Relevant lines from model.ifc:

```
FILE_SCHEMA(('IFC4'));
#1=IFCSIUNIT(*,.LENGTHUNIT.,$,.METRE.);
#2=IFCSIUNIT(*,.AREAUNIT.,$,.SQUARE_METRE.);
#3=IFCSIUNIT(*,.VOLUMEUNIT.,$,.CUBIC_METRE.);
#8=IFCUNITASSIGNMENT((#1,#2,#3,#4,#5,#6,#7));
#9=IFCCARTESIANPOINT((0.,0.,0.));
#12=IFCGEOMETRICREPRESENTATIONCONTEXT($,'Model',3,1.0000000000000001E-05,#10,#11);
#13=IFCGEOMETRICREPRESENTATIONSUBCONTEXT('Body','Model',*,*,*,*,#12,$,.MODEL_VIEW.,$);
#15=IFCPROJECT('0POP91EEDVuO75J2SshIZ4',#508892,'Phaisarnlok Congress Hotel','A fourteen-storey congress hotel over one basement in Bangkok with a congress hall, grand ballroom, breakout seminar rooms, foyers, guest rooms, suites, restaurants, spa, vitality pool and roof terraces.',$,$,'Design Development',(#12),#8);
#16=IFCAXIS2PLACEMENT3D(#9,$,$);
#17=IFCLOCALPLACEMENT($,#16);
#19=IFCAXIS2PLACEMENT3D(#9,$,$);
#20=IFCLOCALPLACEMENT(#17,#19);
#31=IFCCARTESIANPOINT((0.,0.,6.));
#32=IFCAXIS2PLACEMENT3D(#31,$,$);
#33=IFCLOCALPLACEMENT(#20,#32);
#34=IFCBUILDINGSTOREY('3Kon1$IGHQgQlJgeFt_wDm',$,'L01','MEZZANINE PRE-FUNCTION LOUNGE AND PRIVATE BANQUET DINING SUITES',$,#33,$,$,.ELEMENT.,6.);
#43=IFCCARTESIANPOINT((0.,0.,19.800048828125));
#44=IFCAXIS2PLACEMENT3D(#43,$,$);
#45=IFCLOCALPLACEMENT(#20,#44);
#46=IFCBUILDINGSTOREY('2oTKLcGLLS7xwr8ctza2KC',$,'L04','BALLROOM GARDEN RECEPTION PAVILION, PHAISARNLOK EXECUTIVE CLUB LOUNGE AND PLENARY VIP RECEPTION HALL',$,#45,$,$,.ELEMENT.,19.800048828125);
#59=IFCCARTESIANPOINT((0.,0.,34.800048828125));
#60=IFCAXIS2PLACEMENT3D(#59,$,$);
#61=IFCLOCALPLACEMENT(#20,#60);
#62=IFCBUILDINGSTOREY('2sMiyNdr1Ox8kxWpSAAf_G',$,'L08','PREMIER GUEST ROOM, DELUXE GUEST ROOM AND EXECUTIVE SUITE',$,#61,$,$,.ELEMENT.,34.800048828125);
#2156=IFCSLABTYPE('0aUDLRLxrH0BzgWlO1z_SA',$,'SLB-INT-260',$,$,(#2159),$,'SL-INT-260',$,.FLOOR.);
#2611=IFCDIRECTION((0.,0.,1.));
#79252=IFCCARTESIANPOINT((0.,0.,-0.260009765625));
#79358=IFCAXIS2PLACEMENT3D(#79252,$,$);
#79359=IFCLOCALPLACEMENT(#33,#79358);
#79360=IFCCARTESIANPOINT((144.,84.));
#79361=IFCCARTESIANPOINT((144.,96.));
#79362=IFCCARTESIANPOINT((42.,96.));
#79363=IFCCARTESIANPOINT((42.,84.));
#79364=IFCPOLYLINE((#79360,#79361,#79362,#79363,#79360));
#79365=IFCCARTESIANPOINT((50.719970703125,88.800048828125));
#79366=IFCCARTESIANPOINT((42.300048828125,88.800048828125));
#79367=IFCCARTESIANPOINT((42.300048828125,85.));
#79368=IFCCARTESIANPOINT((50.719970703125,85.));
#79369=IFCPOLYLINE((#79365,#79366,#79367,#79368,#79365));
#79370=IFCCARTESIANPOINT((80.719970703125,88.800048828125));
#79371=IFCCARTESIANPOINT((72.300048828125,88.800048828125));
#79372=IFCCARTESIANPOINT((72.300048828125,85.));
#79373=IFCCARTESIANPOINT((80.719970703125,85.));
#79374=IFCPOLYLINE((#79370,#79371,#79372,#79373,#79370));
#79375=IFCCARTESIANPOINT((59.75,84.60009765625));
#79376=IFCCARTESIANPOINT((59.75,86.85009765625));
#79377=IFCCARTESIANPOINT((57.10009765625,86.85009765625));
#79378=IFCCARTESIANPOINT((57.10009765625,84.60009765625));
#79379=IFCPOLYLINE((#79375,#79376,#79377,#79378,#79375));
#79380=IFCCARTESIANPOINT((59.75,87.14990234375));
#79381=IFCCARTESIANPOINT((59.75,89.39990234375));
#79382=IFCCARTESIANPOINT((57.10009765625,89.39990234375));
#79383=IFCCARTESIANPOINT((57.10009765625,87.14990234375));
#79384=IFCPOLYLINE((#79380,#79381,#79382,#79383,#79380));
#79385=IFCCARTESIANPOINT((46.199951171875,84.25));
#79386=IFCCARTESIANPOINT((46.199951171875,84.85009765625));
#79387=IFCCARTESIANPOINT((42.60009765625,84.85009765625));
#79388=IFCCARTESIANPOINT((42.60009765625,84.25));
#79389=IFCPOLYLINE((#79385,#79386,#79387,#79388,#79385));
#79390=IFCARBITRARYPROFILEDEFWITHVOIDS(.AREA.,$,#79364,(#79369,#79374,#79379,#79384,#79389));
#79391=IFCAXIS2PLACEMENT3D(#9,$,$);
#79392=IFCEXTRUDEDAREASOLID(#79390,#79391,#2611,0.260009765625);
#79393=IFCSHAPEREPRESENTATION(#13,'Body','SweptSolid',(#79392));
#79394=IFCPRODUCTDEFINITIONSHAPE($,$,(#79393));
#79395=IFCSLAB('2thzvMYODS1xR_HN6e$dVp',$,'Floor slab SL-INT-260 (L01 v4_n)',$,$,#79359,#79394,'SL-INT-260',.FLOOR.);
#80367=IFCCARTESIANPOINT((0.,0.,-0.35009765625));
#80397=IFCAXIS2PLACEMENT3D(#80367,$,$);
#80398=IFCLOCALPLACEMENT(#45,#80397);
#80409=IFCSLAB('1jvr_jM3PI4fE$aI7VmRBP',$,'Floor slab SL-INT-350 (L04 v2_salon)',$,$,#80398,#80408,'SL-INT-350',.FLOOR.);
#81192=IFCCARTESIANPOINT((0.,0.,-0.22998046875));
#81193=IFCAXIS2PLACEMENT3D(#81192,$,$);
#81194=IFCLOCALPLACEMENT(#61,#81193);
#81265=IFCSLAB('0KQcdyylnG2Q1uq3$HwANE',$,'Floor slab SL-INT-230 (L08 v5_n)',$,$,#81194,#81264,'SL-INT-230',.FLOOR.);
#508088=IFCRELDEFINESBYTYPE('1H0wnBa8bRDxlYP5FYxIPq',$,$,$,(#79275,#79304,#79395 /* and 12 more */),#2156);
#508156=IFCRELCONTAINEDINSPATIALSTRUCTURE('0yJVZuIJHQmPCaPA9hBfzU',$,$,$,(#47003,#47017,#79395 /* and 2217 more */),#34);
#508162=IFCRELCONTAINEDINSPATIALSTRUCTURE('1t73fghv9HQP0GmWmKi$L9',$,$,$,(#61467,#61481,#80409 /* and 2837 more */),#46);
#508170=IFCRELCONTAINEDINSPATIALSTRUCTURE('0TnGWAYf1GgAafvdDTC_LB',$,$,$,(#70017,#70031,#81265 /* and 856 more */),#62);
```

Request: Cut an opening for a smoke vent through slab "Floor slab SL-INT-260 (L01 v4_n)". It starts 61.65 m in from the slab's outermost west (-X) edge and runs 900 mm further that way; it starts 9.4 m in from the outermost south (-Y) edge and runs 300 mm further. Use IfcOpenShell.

```python
import numpy as np
import ifcopenshell
import ifcopenshell.api.feature
import ifcopenshell.api.geometry
import ifcopenshell.api.root
import ifcopenshell.geom
import ifcopenshell.util.placement
import ifcopenshell.util.representation
import ifcopenshell.util.shape
import ifcopenshell.util.unit

model = ifcopenshell.open("model.ifc")
unit_scale = ifcopenshell.util.unit.calculate_unit_scale(model)
settings = ifcopenshell.geom.settings()


def volume(element):
    """Net volume in cubic metres, openings subtracted."""
    shape = ifcopenshell.geom.create_shape(settings, element)
    return ifcopenshell.util.shape.get_volume(shape.geometry)


slab = model.by_guid("2thzvMYODS1xR_HN6e$dVp")
before = volume(slab)

# Extent in the slab's own axes, in metres. The edges named are its -X and -Y sides.
slab_shape = ifcopenshell.geom.create_shape(settings, slab)
vertices = ifcopenshell.util.shape.get_vertices(slab_shape.geometry)
x_min, y_min, bottom = vertices.min(axis=0)
top = vertices[:, 2].max()

opening = ifcopenshell.api.root.create_entity(model, ifc_class="IfcOpeningElement", name="Smoke vent opening", predefined_type="OPENING")
context = ifcopenshell.util.representation.get_context(model, "Model", "Body", "MODEL_VIEW")
width, depth = 0.9, 0.3
outline = [(0.0, 0.0), (width, 0.0), (width, depth), (0.0, depth), (0.0, 0.0)]
# Overshoot both faces by 50 mm so the cut is clean.
shape = ifcopenshell.api.geometry.add_slab_representation(
    model, context=context, depth=top - bottom + 0.1, polyline=outline
)
ifcopenshell.api.geometry.assign_representation(model, product=opening, representation=shape)

matrix = ifcopenshell.util.placement.get_local_placement(slab.ObjectPlacement)
matrix[:, 3] = matrix @ np.append(np.array([x_min + 61.65, y_min + 9.4, bottom - 0.05]) / unit_scale, 1.0)
ifcopenshell.api.geometry.edit_object_placement(model, product=opening, matrix=matrix, is_si=False)
ifcopenshell.api.feature.add_feature(model, feature=opening, element=slab)

after = volume(slab)

print(f"slab volume {before:.3f} -> {after:.3f} m3")

model.write("model_updated.ifc")
```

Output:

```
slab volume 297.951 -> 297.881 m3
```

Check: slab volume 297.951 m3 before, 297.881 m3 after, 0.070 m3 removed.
